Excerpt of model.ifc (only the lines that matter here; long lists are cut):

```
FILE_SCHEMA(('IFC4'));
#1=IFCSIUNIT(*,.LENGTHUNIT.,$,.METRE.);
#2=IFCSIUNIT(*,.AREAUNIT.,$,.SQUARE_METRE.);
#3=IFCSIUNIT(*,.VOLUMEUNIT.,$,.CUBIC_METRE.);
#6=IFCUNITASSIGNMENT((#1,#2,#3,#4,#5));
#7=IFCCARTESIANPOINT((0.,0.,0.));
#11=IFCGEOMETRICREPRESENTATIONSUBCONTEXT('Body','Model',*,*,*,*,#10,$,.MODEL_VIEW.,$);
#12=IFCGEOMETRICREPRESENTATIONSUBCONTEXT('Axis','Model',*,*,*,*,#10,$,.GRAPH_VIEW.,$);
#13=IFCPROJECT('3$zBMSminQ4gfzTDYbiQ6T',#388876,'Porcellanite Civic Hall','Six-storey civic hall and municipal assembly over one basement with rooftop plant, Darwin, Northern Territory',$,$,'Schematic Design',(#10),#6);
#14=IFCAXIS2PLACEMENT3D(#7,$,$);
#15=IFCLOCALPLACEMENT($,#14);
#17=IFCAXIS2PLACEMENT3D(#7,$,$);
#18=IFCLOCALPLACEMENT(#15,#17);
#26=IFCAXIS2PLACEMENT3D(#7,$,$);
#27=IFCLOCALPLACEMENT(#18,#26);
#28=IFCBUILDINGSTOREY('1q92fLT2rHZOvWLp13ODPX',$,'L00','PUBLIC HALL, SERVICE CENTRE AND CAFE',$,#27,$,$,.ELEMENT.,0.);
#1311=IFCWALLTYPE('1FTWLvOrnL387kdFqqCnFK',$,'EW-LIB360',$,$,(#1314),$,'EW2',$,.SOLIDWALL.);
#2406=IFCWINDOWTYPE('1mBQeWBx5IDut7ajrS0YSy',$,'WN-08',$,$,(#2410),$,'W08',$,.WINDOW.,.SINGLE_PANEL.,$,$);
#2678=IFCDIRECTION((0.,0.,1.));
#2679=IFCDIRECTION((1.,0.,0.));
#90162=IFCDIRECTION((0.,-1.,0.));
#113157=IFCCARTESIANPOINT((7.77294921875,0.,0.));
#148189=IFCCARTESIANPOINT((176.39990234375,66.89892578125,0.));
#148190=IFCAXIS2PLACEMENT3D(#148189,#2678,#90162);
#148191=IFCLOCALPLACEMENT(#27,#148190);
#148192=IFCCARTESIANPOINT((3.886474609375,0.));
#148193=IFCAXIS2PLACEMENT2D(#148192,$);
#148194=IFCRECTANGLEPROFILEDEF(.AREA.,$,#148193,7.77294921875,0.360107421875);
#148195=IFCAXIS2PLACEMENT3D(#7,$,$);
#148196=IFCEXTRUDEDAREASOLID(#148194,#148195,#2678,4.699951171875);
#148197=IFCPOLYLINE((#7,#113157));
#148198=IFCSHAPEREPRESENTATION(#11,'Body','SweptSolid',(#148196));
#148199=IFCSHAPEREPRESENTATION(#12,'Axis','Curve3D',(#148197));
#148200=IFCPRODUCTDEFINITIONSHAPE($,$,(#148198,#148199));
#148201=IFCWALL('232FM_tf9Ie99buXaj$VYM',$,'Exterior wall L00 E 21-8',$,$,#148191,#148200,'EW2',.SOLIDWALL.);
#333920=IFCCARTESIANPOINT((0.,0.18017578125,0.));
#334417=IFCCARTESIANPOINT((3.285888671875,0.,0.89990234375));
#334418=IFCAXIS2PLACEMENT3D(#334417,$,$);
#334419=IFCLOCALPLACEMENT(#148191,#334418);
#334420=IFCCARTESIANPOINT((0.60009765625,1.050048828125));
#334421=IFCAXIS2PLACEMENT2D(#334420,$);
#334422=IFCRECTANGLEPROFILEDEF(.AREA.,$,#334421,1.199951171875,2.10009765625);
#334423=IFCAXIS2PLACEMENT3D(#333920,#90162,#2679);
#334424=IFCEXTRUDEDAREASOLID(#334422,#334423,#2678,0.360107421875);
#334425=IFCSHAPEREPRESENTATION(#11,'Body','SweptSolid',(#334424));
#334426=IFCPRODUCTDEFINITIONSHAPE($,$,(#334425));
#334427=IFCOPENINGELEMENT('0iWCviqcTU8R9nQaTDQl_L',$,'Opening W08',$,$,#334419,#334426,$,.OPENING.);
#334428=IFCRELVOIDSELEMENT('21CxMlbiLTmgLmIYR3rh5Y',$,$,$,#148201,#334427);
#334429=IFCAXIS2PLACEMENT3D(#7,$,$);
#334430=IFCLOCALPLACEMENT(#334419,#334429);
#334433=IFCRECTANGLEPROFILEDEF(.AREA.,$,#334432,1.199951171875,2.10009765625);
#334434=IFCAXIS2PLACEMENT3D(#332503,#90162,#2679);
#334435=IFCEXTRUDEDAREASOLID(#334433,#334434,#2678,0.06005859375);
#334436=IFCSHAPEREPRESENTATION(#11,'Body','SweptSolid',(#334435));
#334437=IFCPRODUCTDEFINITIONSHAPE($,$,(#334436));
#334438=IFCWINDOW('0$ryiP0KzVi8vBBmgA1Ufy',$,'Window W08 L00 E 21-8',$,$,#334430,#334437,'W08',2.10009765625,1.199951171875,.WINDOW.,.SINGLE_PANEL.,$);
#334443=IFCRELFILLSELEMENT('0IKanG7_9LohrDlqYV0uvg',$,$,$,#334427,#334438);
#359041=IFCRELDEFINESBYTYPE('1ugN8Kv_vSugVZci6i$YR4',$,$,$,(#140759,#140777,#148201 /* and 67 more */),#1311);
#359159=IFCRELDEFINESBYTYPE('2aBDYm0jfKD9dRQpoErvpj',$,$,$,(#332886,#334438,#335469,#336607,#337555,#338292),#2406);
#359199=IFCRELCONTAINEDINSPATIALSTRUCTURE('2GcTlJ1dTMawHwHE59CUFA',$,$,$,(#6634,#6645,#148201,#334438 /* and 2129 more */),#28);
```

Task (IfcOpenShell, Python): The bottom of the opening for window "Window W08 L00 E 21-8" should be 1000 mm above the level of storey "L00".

```python
import numpy as np
import ifcopenshell
import ifcopenshell.api.geometry
import ifcopenshell.geom
import ifcopenshell.util.element
import ifcopenshell.util.placement
import ifcopenshell.util.shape
import ifcopenshell.util.unit

model = ifcopenshell.open("model.ifc")
unit_scale = ifcopenshell.util.unit.calculate_unit_scale(model)

window = model.by_guid("0$ryiP0KzVi8vBBmgA1Ufy")
opening = window.FillsVoids[0].RelatingOpeningElement
storey = ifcopenshell.util.element.get_container(window, ifc_class="IfcBuildingStorey")
level = ifcopenshell.util.placement.get_local_placement(storey.ObjectPlacement)[2, 3]

# The opening's origin need not be at the sill, so measure its lowest point.
shape = ifcopenshell.geom.create_shape(ifcopenshell.geom.settings(), opening)
bottom = ifcopenshell.util.shape.get_shape_bottom_elevation(shape, shape.geometry) / unit_scale
dz = level + 1.0 - bottom

shift = np.array([0.0, 0.0, dz])
# The window is placed relative to its opening, so it follows when the opening moves.
matrix = ifcopenshell.util.placement.get_local_placement(opening.ObjectPlacement)
matrix[:3, 3] += shift
ifcopenshell.api.geometry.edit_object_placement(
    model, product=opening, matrix=matrix, is_si=False, should_transform_children=True
)

print(f"moved by {dz * unit_scale:+.3f} m")

model.write("model_edited.ifc")
```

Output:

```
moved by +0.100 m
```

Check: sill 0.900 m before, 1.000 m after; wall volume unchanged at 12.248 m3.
